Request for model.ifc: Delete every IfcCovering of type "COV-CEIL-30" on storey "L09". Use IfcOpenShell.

First a look at what the model holds.

```python
import ifcopenshell
import ifcopenshell.util.element

model = ifcopenshell.open("model.ifc")
print(model.schema)
storey = next(s for s in model.by_type("IfcBuildingStorey") if s.Name == "L09")
coverings = [e for e in ifcopenshell.util.element.get_decomposition(storey) if e.is_a("IfcCovering")]
seen = {}
for e in coverings:
    element_type = ifcopenshell.util.element.get_type(e)
    name = element_type.Name if element_type not in (None, e) else None
    seen[name] = seen.get(name, 0) + 1
for name, count in sorted(seen.items(), key=str):
    print(count, "x", name)
```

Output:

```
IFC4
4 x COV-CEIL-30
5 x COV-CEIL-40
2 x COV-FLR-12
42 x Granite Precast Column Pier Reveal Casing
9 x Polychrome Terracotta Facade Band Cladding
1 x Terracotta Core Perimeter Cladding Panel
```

```python
import ifcopenshell
import ifcopenshell.api.root
import ifcopenshell.util.element

model = ifcopenshell.open("model.ifc")

storey = next(s for s in model.by_type("IfcBuildingStorey") if s.Name == "L09")
coverings = [e for e in ifcopenshell.util.element.get_decomposition(storey) if e.is_a("IfcCovering")]
targets = [e for e in coverings if (t := ifcopenshell.util.element.get_type(e)) not in (None, e) and t.Name == "COV-CEIL-30"]

for e in targets:
    ifcopenshell.api.root.remove_product(model, product=e)
print(len(targets), "removed")

model.write("model_v2.ifc")
```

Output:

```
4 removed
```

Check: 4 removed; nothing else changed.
